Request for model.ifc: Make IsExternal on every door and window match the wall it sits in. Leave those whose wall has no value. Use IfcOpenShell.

First a look at what the model holds.

```python
import ifcopenshell
import ifcopenshell.util.element

model = ifcopenshell.open("model.ifc")
print(model.schema)
seen = {}
for e in model.by_type("IfcDoor") + model.by_type("IfcWindow"):
    if not e.FillsVoids:
        continue
    host = e.FillsVoids[0].RelatingOpeningElement.VoidsElements[0].RelatingBuildingElement
    own = ifcopenshell.util.element.get_pset(e, f"Pset_{e.is_a()[3:].removesuffix('StandardCase')}Common", "IsExternal")
    wall = ifcopenshell.util.element.get_pset(host, "Pset_WallCommon", "IsExternal")
    seen[e.is_a(), own, wall] = seen.get((e.is_a(), own, wall), 0) + 1
for (cls, own, wall), count in sorted(seen.items(), key=str):
    print(count, cls, "IsExternal:", own, "| host wall:", wall)
```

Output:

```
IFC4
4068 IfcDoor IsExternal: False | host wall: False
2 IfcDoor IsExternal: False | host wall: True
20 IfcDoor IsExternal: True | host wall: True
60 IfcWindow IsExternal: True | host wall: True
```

```python
import ifcopenshell
import ifcopenshell.api.pset
import ifcopenshell.util.element

model = ifcopenshell.open("model.ifc")

count = 0
for ifc_class, pset_name in (("IfcDoor", "Pset_DoorCommon"), ("IfcWindow", "Pset_WindowCommon")):
    for e in model.by_type(ifc_class):
        if not e.FillsVoids:
            continue
        host = e.FillsVoids[0].RelatingOpeningElement.VoidsElements[0].RelatingBuildingElement
        external = ifcopenshell.util.element.get_pset(host, "Pset_WallCommon", "IsExternal")
        if external is None or ifcopenshell.util.element.get_pset(e, pset_name, "IsExternal") == external:
            continue
        found = ifcopenshell.util.element.get_pset(e, pset_name, should_inherit=False)
        if found:
            pset = model.by_id(found["id"])
            if len(ifcopenshell.util.element.get_elements_by_pset(pset)) > 1:
                pset = ifcopenshell.api.pset.unshare_pset(model, products=[e], pset=pset)[0]
        else:
            pset = ifcopenshell.api.pset.add_pset(model, product=e, name=pset_name)
        ifcopenshell.api.pset.edit_pset(model, pset=pset, properties={"IsExternal": external})
        count += 1

print(count, "updated")

model.write("model_updated.ifc")
```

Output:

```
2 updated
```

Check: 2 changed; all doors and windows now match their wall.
